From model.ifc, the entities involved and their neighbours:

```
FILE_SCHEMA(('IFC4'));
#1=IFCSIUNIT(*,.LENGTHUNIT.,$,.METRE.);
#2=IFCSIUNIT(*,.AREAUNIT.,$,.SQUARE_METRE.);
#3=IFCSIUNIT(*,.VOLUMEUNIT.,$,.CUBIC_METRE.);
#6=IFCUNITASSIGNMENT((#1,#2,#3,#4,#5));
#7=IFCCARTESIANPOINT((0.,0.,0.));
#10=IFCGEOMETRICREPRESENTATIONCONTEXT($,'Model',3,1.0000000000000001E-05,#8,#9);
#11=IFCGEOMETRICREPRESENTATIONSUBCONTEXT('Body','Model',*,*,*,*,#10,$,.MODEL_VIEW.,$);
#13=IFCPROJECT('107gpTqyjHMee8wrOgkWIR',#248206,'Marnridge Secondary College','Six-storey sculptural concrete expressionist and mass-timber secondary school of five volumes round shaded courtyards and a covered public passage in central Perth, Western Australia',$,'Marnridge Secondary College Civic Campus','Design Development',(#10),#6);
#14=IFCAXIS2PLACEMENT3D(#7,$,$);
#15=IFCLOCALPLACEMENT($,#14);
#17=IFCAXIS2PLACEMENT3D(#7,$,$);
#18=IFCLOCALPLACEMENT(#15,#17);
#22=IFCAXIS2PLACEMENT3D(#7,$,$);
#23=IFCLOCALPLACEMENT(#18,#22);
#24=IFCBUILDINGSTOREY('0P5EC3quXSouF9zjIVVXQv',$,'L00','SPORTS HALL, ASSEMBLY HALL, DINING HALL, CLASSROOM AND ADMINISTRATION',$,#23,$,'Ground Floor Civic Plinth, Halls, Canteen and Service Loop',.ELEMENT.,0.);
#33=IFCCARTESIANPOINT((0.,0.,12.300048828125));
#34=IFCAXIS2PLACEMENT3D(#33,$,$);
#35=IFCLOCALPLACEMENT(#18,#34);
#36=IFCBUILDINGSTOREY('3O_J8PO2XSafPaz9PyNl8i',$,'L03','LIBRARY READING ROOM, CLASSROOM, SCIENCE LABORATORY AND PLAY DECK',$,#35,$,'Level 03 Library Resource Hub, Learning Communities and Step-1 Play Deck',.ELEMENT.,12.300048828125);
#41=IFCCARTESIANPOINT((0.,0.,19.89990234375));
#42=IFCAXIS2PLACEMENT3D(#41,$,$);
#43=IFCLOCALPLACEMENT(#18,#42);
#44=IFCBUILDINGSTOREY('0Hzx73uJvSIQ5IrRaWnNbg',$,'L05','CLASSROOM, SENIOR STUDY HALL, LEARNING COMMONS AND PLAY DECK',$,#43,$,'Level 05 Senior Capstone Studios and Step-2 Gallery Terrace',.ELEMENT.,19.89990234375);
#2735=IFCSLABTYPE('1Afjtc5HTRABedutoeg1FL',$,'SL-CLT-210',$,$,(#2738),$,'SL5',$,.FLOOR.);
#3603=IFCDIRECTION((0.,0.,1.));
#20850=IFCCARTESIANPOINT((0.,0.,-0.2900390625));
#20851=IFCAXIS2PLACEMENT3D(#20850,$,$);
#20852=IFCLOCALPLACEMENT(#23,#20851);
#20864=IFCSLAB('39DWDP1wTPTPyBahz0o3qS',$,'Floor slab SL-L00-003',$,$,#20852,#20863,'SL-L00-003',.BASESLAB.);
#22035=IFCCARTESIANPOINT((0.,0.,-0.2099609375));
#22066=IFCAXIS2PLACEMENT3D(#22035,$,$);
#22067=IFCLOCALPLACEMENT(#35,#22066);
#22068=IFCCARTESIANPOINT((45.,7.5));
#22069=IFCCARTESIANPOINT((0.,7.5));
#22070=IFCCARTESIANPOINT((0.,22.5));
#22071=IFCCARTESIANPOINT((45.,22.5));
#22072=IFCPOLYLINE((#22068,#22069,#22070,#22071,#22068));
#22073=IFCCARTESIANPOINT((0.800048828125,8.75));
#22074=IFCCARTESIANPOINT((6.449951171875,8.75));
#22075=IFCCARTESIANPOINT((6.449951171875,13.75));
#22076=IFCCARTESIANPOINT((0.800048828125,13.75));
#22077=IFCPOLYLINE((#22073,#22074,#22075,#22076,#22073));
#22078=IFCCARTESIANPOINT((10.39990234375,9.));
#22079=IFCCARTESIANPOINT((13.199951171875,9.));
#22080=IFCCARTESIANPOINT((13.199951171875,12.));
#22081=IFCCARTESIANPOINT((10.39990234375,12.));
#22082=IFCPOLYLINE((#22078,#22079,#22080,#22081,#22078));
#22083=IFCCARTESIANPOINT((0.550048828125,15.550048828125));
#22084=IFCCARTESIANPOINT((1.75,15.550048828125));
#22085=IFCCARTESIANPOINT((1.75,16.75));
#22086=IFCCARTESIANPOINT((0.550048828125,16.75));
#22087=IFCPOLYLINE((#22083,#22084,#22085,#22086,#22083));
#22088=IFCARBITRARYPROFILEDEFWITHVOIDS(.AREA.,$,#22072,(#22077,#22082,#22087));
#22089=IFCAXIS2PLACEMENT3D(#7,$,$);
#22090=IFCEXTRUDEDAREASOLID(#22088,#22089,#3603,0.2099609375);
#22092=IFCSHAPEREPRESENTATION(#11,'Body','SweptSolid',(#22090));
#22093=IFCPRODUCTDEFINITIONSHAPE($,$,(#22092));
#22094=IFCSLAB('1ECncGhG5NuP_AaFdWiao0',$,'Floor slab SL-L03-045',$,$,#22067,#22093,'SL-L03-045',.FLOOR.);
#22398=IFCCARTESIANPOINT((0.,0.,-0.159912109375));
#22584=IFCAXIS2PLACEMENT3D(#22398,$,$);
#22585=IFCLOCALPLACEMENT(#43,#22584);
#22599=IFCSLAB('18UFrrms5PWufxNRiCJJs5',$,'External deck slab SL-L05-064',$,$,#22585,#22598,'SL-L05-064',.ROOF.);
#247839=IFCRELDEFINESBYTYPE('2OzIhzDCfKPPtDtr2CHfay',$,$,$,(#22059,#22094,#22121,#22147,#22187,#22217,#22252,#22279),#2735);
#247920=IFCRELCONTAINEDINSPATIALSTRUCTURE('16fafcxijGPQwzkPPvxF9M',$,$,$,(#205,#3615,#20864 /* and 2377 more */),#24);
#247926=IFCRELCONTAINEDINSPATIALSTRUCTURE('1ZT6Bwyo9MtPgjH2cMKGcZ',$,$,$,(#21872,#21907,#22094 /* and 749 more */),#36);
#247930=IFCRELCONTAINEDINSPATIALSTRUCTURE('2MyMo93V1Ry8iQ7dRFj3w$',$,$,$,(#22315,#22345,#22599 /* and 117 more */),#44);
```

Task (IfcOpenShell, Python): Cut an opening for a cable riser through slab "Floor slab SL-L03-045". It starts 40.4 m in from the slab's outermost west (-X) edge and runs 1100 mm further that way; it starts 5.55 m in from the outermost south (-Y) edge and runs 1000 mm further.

```python
import numpy as np
import ifcopenshell
import ifcopenshell.api.feature
import ifcopenshell.api.geometry
import ifcopenshell.api.root
import ifcopenshell.geom
import ifcopenshell.util.placement
import ifcopenshell.util.representation
import ifcopenshell.util.shape
import ifcopenshell.util.unit

model = ifcopenshell.open("model.ifc")
unit_scale = ifcopenshell.util.unit.calculate_unit_scale(model)
settings = ifcopenshell.geom.settings()


def volume(element):
    """Net volume in cubic metres, openings subtracted."""
    shape = ifcopenshell.geom.create_shape(settings, element)
    return ifcopenshell.util.shape.get_volume(shape.geometry)


slab = model.by_id(22094)
before = volume(slab)

# Extent in the slab's own axes, in metres. The edges named are its -X and -Y sides.
slab_shape = ifcopenshell.geom.create_shape(settings, slab)
vertices = ifcopenshell.util.shape.get_vertices(slab_shape.geometry)
x_min, y_min, bottom = vertices.min(axis=0)
top = vertices[:, 2].max()

opening = ifcopenshell.api.root.create_entity(model, ifc_class="IfcOpeningElement", name="Cable riser opening", predefined_type="OPENING")
context = ifcopenshell.util.representation.get_context(model, "Model", "Body", "MODEL_VIEW")
width, depth = 1.1, 1
outline = [(0.0, 0.0), (width, 0.0), (width, depth), (0.0, depth), (0.0, 0.0)]
# Overshoot both faces by 50 mm so the cut is clean.
shape = ifcopenshell.api.geometry.add_slab_representation(
    model, context=context, depth=top - bottom + 0.1, polyline=outline
)
ifcopenshell.api.geometry.assign_representation(model, product=opening, representation=shape)

matrix = ifcopenshell.util.placement.get_local_placement(slab.ObjectPlacement)
matrix[:, 3] = matrix @ np.append(np.array([x_min + 40.4, y_min + 5.55, bottom - 0.05]) / unit_scale, 1.0)
ifcopenshell.api.geometry.edit_object_placement(model, product=opening, matrix=matrix, is_si=False)
ifcopenshell.api.feature.add_feature(model, feature=opening, element=slab)

after = volume(slab)

print(f"slab volume {before:.3f} -> {after:.3f} m3")

model.write("model_updated.ifc")
```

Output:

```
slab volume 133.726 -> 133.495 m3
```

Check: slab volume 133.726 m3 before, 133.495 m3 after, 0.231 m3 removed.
